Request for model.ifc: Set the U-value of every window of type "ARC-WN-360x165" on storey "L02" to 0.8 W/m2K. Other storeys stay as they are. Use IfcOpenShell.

First a look at what the model holds.

```python
import ifcopenshell
import ifcopenshell.util.element

model = ifcopenshell.open("model.ifc")
print(model.schema)
storey = next(s for s in model.by_type("IfcBuildingStorey") if s.Name == "L02")
windows = [e for e in ifcopenshell.util.element.get_decomposition(storey) if e.is_a("IfcWindow")]
seen = {}
for e in windows:
    element_type = ifcopenshell.util.element.get_type(e)
    key = (element_type.Name if element_type != e and element_type else None, ifcopenshell.util.element.get_pset(e, "Pset_WindowCommon", "ThermalTransmittance"))
    seen[key] = seen.get(key, 0) + 1
for (name, value), count in sorted(seen.items(), key=str):
    print(count, "x", name, "|", value)
```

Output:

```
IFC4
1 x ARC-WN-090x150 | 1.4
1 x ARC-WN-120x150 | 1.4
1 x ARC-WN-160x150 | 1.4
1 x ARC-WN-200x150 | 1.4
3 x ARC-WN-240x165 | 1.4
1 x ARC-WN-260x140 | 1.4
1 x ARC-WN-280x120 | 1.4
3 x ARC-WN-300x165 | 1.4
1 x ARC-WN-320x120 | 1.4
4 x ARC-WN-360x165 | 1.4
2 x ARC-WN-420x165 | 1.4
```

```python
import ifcopenshell
import ifcopenshell.api.pset
import ifcopenshell.util.element

model = ifcopenshell.open("model.ifc")

storey = next(s for s in model.by_type("IfcBuildingStorey") if s.Name == "L02")
windows = [e for e in ifcopenshell.util.element.get_decomposition(storey) if e.is_a("IfcWindow")]

count = 0
for e in windows:
    element_type = ifcopenshell.util.element.get_type(e)
    if element_type in (None, e) or element_type.Name != "ARC-WN-360x165":
        continue
    # add_pset returns the element's existing set when there is one.
    pset = ifcopenshell.api.pset.add_pset(model, product=e, name="Pset_WindowCommon")
    ifcopenshell.api.pset.edit_pset(model, pset=pset, properties={"ThermalTransmittance": 0.8})
    count += 1

print(count, "windows updated")

model.write("model_rev.ifc")
```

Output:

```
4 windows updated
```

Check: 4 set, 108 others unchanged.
